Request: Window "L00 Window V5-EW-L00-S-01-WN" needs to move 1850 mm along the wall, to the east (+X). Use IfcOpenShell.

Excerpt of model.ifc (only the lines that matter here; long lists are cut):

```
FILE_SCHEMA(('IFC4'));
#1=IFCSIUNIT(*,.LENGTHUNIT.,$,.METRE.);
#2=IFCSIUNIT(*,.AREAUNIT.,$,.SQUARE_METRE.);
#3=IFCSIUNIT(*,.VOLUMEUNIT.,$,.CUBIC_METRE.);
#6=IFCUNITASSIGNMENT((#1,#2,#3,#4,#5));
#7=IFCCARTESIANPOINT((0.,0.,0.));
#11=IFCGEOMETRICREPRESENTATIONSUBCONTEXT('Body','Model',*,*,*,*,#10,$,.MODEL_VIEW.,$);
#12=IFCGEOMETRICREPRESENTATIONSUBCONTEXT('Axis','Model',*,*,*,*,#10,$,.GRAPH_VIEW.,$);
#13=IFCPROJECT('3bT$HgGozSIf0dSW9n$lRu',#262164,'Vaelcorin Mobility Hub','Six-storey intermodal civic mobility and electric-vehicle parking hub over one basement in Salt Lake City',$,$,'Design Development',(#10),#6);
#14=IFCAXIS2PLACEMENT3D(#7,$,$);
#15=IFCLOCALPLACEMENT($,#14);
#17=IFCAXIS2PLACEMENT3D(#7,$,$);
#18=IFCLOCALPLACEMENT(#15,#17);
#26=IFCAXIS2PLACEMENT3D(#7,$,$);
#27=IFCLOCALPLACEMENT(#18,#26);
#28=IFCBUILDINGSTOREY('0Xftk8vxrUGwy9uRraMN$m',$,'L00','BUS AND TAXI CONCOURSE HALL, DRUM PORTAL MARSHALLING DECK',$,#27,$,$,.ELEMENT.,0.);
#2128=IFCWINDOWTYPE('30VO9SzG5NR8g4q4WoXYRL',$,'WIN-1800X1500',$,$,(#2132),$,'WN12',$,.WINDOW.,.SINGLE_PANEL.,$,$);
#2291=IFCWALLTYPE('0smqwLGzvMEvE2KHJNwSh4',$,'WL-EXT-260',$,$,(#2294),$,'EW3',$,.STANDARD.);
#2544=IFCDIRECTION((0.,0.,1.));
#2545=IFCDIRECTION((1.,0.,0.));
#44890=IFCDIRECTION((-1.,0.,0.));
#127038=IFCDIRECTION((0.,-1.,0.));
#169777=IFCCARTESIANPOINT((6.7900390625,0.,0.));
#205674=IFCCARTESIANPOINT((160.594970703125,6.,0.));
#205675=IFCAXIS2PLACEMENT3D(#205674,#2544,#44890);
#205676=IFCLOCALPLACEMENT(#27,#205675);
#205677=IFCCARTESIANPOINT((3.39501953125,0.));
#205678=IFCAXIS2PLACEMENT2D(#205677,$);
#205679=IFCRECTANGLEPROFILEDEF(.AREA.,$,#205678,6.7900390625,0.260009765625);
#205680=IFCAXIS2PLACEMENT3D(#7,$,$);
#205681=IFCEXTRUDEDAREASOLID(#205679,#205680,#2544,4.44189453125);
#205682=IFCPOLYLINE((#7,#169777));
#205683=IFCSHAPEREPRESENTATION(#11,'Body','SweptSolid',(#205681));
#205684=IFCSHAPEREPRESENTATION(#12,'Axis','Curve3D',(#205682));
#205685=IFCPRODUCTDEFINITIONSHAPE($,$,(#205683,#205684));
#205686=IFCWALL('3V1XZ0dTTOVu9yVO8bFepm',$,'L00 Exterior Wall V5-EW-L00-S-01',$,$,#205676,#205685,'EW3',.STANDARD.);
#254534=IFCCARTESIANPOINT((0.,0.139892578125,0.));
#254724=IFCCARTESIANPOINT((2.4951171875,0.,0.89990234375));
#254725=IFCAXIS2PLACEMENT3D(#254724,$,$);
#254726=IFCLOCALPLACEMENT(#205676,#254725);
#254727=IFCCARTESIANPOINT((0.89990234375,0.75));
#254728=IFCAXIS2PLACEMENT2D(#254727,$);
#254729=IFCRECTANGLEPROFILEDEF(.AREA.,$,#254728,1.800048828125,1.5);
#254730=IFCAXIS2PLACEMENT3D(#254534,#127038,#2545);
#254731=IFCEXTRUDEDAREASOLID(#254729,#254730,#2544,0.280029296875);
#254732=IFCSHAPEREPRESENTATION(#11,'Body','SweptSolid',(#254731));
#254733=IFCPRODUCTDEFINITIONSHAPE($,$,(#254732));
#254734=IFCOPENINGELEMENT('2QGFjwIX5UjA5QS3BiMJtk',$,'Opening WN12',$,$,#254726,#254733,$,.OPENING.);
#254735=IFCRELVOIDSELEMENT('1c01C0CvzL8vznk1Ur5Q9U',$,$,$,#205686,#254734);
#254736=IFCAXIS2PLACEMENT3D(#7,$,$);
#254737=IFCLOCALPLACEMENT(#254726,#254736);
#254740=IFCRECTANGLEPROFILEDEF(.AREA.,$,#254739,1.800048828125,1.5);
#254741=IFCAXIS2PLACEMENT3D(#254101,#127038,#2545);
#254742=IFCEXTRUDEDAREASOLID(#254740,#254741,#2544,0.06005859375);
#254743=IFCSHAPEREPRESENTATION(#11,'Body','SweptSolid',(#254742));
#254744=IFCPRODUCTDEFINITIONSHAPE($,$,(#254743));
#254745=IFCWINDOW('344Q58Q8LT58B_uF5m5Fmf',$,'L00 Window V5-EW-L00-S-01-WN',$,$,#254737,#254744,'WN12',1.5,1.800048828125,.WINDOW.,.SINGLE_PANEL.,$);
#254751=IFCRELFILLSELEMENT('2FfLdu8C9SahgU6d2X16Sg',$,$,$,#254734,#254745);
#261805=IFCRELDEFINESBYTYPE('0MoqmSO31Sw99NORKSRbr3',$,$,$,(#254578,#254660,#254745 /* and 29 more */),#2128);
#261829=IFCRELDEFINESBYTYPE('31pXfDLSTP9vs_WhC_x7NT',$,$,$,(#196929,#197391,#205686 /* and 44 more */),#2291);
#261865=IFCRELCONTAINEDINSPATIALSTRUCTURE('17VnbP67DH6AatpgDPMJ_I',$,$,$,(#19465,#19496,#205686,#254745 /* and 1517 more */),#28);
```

```python
import ifcopenshell
import ifcopenshell.api.geometry
import ifcopenshell.util.placement

model = ifcopenshell.open("model.ifc")

window = model.by_guid("344Q58Q8LT58B_uF5m5Fmf")
opening = window.FillsVoids[0].RelatingOpeningElement
wall = opening.VoidsElements[0].RelatingBuildingElement

wall_matrix = ifcopenshell.util.placement.get_local_placement(wall.ObjectPlacement)
shift = wall_matrix[:3, 0] * -1.85
before = ifcopenshell.util.placement.get_local_placement(window.ObjectPlacement)[:3, 3].copy()

# The window is placed relative to its opening, so it follows when the opening moves.
matrix = ifcopenshell.util.placement.get_local_placement(opening.ObjectPlacement)
matrix[:3, 3] += shift
ifcopenshell.api.geometry.edit_object_placement(
    model, product=opening, matrix=matrix, is_si=False, should_transform_children=True
)

after = ifcopenshell.util.placement.get_local_placement(window.ObjectPlacement)[:3, 3]
print("window moved by", (after - before).round(3) + 0.0)

model.write("model_rev.ifc")
```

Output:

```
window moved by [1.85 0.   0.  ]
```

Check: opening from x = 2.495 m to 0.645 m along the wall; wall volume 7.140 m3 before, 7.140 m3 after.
